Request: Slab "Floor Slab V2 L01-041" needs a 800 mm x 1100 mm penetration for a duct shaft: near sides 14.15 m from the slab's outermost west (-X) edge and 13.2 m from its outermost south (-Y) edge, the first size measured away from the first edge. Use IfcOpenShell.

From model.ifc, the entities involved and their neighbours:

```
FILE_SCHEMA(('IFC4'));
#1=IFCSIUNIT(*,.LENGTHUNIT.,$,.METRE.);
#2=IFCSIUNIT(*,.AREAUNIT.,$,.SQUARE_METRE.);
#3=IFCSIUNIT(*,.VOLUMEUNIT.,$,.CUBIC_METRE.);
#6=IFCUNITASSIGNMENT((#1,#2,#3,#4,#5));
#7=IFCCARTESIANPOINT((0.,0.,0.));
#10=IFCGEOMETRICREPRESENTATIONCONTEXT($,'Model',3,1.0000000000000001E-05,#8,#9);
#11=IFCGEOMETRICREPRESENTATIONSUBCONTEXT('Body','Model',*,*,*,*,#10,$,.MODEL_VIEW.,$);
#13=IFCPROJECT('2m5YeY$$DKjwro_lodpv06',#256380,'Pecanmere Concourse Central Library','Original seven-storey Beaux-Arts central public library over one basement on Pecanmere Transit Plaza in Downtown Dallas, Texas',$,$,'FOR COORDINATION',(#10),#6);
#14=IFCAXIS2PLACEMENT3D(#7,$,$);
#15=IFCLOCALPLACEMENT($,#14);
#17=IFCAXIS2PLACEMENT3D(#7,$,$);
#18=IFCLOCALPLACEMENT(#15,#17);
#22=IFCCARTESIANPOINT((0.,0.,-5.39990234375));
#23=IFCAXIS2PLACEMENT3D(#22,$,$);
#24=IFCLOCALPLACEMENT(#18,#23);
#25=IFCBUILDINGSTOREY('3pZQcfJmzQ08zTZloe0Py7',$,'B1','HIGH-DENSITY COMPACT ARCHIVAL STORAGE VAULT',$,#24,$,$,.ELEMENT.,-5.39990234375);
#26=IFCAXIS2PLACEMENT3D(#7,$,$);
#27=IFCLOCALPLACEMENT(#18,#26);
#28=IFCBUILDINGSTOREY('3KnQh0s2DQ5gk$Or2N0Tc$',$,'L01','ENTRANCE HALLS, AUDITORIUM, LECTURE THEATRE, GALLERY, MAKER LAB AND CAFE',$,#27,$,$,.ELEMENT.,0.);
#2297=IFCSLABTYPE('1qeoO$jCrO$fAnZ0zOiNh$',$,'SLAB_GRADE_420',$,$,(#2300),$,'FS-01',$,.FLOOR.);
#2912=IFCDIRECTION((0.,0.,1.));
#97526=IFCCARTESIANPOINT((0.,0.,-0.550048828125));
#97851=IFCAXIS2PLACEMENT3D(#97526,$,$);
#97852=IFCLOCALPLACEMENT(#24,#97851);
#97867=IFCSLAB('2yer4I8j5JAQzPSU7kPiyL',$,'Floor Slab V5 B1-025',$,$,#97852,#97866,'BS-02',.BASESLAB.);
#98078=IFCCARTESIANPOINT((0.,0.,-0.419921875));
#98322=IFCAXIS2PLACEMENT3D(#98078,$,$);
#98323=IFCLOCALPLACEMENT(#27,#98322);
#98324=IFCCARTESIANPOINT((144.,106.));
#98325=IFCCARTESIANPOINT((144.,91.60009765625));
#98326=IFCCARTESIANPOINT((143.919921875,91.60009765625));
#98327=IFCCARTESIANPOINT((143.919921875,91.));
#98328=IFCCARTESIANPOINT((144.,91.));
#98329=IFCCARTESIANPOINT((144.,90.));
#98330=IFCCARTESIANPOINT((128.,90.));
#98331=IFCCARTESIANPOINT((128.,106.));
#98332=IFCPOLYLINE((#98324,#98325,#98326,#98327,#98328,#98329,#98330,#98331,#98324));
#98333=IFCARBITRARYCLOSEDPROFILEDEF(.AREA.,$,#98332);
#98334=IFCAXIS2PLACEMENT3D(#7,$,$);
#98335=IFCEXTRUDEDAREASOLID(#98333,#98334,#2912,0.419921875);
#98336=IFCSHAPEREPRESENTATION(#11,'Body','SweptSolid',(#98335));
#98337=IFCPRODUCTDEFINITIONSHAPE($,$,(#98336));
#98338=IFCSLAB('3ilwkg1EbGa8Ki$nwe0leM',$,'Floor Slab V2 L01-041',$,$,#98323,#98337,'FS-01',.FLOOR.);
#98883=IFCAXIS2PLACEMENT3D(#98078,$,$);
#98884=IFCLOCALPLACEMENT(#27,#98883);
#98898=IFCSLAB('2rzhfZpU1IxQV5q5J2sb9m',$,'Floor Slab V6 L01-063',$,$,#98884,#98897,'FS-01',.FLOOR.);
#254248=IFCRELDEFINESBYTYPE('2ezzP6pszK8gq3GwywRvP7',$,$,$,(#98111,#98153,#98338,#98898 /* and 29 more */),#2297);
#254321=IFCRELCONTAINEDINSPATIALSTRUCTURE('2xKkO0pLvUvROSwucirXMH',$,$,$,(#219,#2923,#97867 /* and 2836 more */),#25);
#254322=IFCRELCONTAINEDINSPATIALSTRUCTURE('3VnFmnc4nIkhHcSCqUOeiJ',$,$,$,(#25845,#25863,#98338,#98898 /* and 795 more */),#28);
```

```python
import numpy as np
import ifcopenshell
import ifcopenshell.api.feature
import ifcopenshell.api.geometry
import ifcopenshell.api.root
import ifcopenshell.geom
import ifcopenshell.util.placement
import ifcopenshell.util.representation
import ifcopenshell.util.shape
import ifcopenshell.util.unit

model = ifcopenshell.open("model.ifc")
unit_scale = ifcopenshell.util.unit.calculate_unit_scale(model)
settings = ifcopenshell.geom.settings()


def volume(element):
    """Net volume in cubic metres, openings subtracted."""
    shape = ifcopenshell.geom.create_shape(settings, element)
    return ifcopenshell.util.shape.get_volume(shape.geometry)


slab = model.by_guid("3ilwkg1EbGa8Ki$nwe0leM")
before = volume(slab)

# Extent in the slab's own axes, in metres. The edges named are its -X and -Y sides.
slab_shape = ifcopenshell.geom.create_shape(settings, slab)
vertices = ifcopenshell.util.shape.get_vertices(slab_shape.geometry)
x_min, y_min, bottom = vertices.min(axis=0)
top = vertices[:, 2].max()

opening = ifcopenshell.api.root.create_entity(model, ifc_class="IfcOpeningElement", name="Duct shaft opening", predefined_type="OPENING")
context = ifcopenshell.util.representation.get_context(model, "Model", "Body", "MODEL_VIEW")
width, depth = 0.8, 1.1
outline = [(0.0, 0.0), (width, 0.0), (width, depth), (0.0, depth), (0.0, 0.0)]
# Overshoot both faces by 50 mm so the cut is clean.
shape = ifcopenshell.api.geometry.add_slab_representation(
    model, context=context, depth=top - bottom + 0.1, polyline=outline
)
ifcopenshell.api.geometry.assign_representation(model, product=opening, representation=shape)

matrix = ifcopenshell.util.placement.get_local_placement(slab.ObjectPlacement)
matrix[:, 3] = matrix @ np.append(np.array([x_min + 14.15, y_min + 13.2, bottom - 0.05]) / unit_scale, 1.0)
ifcopenshell.api.geometry.edit_object_placement(model, product=opening, matrix=matrix, is_si=False)
ifcopenshell.api.feature.add_feature(model, feature=opening, element=slab)

after = volume(slab)

print(f"slab volume {before:.3f} -> {after:.3f} m3")

model.write("model_updated.ifc")
```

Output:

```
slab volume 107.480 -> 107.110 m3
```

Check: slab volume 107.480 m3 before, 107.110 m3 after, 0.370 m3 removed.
